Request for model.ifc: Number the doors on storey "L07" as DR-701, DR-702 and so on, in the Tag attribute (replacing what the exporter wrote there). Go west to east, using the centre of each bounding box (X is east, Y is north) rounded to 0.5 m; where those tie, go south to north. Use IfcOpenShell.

First a look at what the model holds.

```python
import ifcopenshell
import ifcopenshell.util.element
import ifcopenshell.util.placement

model = ifcopenshell.open("model.ifc")
print(model.schema)
storey = next(s for s in model.by_type("IfcBuildingStorey") if s.Name == "L07")
doors = [e for e in ifcopenshell.util.element.get_decomposition(storey) if e.is_a("IfcDoor")]
for e in sorted(doors, key=lambda e: e.id()):
    origin = ifcopenshell.util.placement.get_local_placement(e.ObjectPlacement)[:3, 3]
    print(e.id(), e.Tag, e.Name, origin.round(2) + 0.0, sep=" | ")
```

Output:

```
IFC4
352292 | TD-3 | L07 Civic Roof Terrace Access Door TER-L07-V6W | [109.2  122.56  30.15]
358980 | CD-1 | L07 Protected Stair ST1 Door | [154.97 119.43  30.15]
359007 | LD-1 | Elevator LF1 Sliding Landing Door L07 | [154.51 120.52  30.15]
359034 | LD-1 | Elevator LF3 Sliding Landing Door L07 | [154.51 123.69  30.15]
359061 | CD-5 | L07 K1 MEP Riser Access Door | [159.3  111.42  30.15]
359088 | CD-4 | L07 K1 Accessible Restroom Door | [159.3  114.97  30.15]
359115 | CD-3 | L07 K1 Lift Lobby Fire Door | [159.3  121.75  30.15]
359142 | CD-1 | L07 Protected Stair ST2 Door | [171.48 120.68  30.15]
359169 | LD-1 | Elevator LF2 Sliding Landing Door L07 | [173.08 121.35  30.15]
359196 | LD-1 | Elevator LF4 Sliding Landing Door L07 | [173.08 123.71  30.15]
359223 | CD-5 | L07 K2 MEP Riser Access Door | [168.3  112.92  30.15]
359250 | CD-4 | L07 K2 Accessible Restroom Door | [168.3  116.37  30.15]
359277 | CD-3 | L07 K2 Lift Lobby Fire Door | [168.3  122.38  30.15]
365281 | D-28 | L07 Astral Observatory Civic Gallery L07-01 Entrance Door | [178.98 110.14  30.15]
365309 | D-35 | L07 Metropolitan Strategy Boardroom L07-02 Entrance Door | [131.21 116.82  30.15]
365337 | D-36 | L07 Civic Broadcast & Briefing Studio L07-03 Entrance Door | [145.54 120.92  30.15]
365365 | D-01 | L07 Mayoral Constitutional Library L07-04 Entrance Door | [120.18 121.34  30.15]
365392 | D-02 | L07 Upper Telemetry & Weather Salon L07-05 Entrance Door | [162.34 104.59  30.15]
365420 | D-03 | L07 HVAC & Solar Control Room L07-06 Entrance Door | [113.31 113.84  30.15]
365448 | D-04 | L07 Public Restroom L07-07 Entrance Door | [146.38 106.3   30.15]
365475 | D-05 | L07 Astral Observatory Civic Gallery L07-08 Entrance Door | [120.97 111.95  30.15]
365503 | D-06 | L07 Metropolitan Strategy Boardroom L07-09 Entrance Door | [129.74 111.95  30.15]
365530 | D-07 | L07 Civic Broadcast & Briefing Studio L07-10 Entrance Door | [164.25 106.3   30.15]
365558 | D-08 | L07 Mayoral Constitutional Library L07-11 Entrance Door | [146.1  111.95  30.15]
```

```python
import ifcopenshell
import ifcopenshell.geom
import ifcopenshell.util.element
import ifcopenshell.util.shape

model = ifcopenshell.open("model.ifc")
settings = ifcopenshell.geom.settings()
settings.set("use-world-coords", True)


def centre(element):
    shape = ifcopenshell.geom.create_shape(settings, element)
    return ifcopenshell.util.shape.get_bbox_centroid(shape.geometry)


storey = next(s for s in model.by_type("IfcBuildingStorey") if s.Name == "L07")
doors = [e for e in ifcopenshell.util.element.get_decomposition(storey) if e.is_a("IfcDoor")]

# Insertion points can sit at a corner or the storey origin, so sort by the geometry (in metres).
centres = {e: centre(e) for e in doors}
doors.sort(key=lambda e: (round(centres[e][0] / 0.5), centres[e][1]))

for i, e in enumerate(doors, start=1):
    number = f"DR-7{i:02d}"
    e.Tag = number
    print(e.id(), number)

model.write("model_v2.ifc")
```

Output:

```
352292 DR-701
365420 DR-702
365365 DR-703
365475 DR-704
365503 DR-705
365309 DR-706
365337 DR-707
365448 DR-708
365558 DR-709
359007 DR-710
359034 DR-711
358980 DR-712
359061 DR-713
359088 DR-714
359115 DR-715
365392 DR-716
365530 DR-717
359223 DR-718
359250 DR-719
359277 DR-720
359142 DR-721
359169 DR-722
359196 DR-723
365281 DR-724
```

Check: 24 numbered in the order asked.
